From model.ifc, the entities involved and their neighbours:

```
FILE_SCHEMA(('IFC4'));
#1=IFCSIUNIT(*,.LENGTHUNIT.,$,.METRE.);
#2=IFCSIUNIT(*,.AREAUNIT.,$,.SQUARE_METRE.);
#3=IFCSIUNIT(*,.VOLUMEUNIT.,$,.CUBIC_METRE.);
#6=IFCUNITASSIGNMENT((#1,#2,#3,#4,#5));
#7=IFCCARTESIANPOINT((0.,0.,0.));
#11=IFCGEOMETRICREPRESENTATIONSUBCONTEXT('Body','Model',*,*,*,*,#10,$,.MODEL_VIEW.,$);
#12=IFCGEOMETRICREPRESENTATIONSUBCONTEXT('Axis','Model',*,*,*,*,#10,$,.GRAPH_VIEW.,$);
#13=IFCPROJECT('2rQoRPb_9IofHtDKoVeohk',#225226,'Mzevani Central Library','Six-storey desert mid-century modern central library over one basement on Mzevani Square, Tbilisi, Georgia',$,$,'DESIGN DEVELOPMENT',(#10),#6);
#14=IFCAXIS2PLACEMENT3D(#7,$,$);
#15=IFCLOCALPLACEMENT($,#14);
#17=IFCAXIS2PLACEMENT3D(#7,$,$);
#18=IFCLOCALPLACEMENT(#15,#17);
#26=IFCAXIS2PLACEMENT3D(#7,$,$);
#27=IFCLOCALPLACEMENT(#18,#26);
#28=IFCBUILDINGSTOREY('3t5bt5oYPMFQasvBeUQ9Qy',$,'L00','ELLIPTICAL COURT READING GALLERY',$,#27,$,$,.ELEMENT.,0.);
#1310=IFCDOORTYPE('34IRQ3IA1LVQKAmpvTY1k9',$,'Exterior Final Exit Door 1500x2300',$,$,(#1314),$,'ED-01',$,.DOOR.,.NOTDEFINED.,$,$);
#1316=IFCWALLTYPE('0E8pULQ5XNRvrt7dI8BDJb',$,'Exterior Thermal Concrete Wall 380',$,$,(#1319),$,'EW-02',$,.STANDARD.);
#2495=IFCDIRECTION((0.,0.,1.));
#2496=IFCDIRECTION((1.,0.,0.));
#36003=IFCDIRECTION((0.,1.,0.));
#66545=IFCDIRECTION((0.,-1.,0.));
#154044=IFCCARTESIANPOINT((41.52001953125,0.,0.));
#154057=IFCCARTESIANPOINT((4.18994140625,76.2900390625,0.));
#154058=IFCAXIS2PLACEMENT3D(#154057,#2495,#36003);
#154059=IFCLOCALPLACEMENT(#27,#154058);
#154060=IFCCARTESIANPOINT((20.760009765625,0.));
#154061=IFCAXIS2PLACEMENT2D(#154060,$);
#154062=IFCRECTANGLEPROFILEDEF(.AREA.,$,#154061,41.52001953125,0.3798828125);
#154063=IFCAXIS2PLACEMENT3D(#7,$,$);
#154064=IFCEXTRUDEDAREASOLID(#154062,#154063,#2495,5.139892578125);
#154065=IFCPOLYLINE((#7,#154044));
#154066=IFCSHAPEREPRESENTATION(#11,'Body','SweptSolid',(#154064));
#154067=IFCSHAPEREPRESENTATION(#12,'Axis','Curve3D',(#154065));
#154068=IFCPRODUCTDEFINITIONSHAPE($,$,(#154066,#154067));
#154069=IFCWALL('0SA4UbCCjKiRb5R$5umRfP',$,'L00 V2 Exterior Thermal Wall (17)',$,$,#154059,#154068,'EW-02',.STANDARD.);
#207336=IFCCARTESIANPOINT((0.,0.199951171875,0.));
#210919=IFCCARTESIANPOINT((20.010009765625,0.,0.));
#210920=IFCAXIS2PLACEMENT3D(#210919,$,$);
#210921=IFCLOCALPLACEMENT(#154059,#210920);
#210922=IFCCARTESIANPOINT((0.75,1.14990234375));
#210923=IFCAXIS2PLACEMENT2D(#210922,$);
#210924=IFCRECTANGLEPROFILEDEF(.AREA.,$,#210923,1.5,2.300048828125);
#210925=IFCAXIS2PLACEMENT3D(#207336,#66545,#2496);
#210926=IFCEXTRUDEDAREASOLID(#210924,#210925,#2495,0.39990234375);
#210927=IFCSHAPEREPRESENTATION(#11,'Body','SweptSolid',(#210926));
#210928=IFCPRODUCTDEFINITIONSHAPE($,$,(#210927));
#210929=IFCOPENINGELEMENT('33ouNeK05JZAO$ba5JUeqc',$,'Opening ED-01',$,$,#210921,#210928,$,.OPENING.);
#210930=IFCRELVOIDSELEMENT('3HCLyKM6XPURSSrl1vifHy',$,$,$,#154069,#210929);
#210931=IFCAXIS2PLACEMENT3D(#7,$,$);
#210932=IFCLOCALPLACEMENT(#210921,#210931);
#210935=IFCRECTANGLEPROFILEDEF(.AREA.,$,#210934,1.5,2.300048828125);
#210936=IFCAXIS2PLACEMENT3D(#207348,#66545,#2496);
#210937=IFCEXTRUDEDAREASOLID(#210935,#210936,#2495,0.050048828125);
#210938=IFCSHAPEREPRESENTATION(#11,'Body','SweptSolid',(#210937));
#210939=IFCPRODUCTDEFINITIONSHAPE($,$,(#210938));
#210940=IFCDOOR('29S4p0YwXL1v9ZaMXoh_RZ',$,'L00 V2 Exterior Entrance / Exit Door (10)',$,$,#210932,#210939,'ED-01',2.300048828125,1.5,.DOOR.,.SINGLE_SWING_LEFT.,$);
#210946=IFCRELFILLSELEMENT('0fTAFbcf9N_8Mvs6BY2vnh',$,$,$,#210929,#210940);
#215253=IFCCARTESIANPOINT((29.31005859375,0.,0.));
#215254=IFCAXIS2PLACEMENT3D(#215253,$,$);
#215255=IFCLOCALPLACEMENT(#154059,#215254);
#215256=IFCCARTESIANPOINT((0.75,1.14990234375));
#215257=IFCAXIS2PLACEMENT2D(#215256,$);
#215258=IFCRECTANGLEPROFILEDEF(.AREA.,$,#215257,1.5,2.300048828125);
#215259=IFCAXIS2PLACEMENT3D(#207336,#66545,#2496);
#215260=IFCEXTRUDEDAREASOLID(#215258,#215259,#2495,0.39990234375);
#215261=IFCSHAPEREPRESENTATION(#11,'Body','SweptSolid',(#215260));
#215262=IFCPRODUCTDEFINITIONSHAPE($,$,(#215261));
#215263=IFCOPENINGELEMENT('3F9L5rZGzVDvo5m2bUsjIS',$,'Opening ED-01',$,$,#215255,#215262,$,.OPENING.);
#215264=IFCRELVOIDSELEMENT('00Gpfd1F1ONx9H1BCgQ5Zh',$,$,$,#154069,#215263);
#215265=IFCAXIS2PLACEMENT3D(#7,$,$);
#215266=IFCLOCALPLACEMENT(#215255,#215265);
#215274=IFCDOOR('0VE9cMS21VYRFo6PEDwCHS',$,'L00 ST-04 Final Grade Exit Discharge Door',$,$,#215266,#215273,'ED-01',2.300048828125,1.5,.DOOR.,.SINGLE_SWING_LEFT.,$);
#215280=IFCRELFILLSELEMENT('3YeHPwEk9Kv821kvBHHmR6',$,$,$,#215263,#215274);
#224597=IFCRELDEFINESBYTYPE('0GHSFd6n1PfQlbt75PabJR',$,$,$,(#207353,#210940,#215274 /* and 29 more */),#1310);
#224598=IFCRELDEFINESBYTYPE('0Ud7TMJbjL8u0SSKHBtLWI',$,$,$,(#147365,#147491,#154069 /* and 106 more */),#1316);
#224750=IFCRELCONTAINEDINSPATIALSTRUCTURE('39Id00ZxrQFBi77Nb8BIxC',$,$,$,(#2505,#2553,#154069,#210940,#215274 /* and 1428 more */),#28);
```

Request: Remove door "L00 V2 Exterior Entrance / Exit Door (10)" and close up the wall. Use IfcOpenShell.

```python
import ifcopenshell
import ifcopenshell.api.feature
import ifcopenshell.api.root
import ifcopenshell.geom
import ifcopenshell.util.shape

model = ifcopenshell.open("model.ifc")
settings = ifcopenshell.geom.settings()


def volume(element):
    """Net volume in cubic metres, openings subtracted."""
    shape = ifcopenshell.geom.create_shape(settings, element)
    return ifcopenshell.util.shape.get_volume(shape.geometry)


door = model.by_guid("29S4p0YwXL1v9ZaMXoh_RZ")
opening = door.FillsVoids[0].RelatingOpeningElement
wall = opening.VoidsElements[0].RelatingBuildingElement
before = volume(wall)

ifcopenshell.api.root.remove_product(model, product=door)
ifcopenshell.api.feature.remove_feature(model, feature=opening)

after = volume(wall)

print(f"wall volume {before:.3f} -> {after:.3f} m3")

model.write("model_edited.ifc")
```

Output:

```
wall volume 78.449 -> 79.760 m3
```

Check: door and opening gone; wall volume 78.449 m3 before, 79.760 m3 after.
